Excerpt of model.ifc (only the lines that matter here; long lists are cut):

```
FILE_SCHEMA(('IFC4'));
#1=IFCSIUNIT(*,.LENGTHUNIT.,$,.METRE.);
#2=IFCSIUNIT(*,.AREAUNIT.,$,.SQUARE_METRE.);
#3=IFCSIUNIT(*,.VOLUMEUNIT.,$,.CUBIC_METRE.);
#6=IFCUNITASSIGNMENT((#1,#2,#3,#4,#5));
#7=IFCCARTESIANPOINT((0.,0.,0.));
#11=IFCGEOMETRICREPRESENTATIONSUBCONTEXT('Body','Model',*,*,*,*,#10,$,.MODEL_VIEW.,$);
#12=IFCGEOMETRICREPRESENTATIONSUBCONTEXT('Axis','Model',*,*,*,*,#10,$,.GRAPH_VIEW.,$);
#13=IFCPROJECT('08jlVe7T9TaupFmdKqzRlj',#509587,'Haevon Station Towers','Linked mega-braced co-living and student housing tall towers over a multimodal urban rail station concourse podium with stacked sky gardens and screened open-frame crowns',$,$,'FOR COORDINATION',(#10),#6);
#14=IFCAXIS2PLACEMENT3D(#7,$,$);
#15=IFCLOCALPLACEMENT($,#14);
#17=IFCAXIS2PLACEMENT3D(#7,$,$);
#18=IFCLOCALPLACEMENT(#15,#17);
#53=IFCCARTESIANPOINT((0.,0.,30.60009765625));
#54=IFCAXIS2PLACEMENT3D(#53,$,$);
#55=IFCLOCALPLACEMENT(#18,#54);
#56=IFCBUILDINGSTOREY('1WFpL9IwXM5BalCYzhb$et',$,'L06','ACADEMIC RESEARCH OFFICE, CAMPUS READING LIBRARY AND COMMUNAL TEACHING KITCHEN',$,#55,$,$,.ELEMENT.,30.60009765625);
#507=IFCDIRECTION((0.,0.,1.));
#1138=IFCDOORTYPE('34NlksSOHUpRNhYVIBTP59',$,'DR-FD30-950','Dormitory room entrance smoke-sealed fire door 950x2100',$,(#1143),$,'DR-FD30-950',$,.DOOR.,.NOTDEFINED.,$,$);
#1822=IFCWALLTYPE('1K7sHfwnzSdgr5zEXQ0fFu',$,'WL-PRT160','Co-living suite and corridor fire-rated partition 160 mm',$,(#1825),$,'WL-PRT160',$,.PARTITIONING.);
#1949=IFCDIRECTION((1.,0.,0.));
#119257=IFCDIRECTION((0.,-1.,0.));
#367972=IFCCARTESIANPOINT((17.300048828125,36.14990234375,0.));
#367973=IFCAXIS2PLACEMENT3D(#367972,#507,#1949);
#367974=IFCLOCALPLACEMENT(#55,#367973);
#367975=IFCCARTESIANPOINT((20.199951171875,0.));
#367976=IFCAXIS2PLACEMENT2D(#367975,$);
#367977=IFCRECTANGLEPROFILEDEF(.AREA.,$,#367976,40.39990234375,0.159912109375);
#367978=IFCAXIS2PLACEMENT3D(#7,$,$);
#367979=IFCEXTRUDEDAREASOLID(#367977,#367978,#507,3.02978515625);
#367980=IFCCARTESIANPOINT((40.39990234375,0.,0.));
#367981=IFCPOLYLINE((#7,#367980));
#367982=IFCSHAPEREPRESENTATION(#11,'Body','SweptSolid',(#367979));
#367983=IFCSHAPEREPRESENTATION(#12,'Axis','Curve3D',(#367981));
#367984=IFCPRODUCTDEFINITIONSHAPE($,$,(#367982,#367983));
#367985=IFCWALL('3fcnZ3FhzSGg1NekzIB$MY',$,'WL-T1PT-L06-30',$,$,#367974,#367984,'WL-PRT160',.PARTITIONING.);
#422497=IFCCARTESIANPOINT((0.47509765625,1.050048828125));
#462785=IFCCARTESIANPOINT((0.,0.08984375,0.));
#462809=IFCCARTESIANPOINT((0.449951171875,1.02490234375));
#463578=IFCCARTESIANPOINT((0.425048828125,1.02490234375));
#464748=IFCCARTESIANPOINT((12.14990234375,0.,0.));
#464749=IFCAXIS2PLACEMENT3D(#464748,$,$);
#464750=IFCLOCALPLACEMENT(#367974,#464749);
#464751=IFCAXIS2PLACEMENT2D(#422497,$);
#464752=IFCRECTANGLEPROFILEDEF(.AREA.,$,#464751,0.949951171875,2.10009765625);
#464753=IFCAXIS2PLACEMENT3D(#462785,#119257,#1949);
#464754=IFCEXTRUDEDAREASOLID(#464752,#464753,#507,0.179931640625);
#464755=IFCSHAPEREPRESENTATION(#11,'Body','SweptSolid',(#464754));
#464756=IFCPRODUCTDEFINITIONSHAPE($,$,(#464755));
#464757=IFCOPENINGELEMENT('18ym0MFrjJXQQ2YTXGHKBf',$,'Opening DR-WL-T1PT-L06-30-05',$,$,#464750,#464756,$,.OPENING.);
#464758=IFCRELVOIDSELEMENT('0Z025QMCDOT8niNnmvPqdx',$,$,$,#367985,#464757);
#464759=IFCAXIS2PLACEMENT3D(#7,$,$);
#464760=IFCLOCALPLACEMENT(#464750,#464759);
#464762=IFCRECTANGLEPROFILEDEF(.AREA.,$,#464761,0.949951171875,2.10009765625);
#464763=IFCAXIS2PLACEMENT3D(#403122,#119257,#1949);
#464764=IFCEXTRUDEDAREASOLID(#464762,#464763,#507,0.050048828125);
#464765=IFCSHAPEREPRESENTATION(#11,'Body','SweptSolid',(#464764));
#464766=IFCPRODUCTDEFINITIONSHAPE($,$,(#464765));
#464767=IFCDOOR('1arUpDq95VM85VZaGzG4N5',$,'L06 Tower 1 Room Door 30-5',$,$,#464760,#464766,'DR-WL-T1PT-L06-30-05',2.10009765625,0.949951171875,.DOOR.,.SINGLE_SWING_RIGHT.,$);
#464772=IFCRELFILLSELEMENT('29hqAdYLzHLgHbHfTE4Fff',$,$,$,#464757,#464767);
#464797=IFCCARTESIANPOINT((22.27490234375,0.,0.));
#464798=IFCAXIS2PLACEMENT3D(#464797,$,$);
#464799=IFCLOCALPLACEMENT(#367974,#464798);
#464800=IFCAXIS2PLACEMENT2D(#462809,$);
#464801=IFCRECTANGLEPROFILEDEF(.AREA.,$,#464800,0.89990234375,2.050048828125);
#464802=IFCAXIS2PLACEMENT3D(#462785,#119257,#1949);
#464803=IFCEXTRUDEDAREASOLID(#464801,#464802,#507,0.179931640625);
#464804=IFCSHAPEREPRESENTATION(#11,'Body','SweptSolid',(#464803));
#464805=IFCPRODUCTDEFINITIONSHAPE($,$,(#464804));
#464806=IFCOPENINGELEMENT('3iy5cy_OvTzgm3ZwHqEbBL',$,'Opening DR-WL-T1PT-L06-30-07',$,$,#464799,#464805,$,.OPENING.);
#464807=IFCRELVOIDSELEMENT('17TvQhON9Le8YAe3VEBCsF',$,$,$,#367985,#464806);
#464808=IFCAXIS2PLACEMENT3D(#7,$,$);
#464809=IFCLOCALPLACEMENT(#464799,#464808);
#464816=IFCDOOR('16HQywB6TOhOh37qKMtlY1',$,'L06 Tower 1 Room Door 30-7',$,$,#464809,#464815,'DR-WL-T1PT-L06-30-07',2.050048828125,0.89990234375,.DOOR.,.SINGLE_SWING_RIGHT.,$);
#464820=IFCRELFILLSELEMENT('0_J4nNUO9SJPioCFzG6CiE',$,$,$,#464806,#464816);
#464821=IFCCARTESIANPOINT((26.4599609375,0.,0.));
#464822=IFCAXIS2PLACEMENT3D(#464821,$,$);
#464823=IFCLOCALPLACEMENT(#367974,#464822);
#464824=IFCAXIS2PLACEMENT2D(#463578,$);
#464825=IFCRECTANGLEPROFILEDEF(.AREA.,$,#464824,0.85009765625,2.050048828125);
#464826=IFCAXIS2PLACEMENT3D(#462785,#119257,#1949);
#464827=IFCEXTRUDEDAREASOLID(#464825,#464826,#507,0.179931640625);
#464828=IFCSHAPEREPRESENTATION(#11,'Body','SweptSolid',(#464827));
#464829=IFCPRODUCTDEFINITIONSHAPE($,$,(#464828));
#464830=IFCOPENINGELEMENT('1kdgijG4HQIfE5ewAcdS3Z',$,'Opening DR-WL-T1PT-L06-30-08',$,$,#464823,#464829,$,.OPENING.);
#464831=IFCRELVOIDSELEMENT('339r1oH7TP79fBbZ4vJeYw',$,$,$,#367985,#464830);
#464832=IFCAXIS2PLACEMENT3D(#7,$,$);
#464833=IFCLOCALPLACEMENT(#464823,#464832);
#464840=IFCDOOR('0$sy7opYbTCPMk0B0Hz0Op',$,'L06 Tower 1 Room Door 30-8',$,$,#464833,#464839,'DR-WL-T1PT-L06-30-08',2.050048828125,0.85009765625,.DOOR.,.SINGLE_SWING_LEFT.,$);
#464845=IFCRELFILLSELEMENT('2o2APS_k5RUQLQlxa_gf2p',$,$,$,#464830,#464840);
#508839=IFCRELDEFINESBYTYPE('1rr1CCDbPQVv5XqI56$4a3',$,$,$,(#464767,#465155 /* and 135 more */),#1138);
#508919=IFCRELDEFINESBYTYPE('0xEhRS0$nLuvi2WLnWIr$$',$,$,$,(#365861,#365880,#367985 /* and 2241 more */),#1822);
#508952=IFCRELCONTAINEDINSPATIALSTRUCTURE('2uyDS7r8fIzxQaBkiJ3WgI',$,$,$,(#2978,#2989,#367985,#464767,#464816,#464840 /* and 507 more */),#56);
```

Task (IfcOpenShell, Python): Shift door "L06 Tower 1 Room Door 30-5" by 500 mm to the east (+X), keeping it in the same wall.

```python
import ifcopenshell
import ifcopenshell.api.geometry
import ifcopenshell.util.placement

model = ifcopenshell.open("model.ifc")

door = model.by_id(464767)
opening = door.FillsVoids[0].RelatingOpeningElement
wall = opening.VoidsElements[0].RelatingBuildingElement

wall_matrix = ifcopenshell.util.placement.get_local_placement(wall.ObjectPlacement)
shift = wall_matrix[:3, 0] * 0.5
before = ifcopenshell.util.placement.get_local_placement(door.ObjectPlacement)[:3, 3].copy()

# The door is placed relative to its opening, so it follows when the opening moves.
matrix = ifcopenshell.util.placement.get_local_placement(opening.ObjectPlacement)
matrix[:3, 3] += shift
ifcopenshell.api.geometry.edit_object_placement(
    model, product=opening, matrix=matrix, is_si=False, should_transform_children=True
)

after = ifcopenshell.util.placement.get_local_placement(door.ObjectPlacement)[:3, 3]
print("door moved by", (after - before).round(3) + 0.0)

model.write("model_edited.ifc")
```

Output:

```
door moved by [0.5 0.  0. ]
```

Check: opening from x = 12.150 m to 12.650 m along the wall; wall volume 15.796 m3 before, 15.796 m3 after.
